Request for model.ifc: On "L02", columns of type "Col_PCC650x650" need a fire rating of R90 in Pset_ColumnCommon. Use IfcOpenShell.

First a look at what the model holds.

```python
import ifcopenshell
import ifcopenshell.util.element

model = ifcopenshell.open("model.ifc")
print(model.schema)
storey = next(s for s in model.by_type("IfcBuildingStorey") if s.Name == "L02")
columns = [e for e in ifcopenshell.util.element.get_decomposition(storey) if e.is_a("IfcColumn")]
seen = {}
for e in columns:
    element_type = ifcopenshell.util.element.get_type(e)
    key = (element_type.Name if element_type != e and element_type else None, ifcopenshell.util.element.get_pset(e, "Pset_ColumnCommon", "FireRating"))
    seen[key] = seen.get(key, 0) + 1
for (name, value), count in sorted(seen.items(), key=str):
    print(count, "x", name, "|", value)
```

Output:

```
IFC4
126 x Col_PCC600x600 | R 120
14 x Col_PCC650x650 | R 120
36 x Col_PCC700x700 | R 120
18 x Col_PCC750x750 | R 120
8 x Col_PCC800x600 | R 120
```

```python
import ifcopenshell
import ifcopenshell.api.pset
import ifcopenshell.util.element

model = ifcopenshell.open("model.ifc")

storey = next(s for s in model.by_type("IfcBuildingStorey") if s.Name == "L02")
columns = [e for e in ifcopenshell.util.element.get_decomposition(storey) if e.is_a("IfcColumn")]

count = 0
for e in columns:
    element_type = ifcopenshell.util.element.get_type(e)
    if element_type in (None, e) or element_type.Name != "Col_PCC650x650":
        continue
    # add_pset returns the element's existing set when there is one.
    pset = ifcopenshell.api.pset.add_pset(model, product=e, name="Pset_ColumnCommon")
    ifcopenshell.api.pset.edit_pset(model, pset=pset, properties={"FireRating": "R90"})
    count += 1

print(count, "columns updated")

model.write("model_rev.ifc")
```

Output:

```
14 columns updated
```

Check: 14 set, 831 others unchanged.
